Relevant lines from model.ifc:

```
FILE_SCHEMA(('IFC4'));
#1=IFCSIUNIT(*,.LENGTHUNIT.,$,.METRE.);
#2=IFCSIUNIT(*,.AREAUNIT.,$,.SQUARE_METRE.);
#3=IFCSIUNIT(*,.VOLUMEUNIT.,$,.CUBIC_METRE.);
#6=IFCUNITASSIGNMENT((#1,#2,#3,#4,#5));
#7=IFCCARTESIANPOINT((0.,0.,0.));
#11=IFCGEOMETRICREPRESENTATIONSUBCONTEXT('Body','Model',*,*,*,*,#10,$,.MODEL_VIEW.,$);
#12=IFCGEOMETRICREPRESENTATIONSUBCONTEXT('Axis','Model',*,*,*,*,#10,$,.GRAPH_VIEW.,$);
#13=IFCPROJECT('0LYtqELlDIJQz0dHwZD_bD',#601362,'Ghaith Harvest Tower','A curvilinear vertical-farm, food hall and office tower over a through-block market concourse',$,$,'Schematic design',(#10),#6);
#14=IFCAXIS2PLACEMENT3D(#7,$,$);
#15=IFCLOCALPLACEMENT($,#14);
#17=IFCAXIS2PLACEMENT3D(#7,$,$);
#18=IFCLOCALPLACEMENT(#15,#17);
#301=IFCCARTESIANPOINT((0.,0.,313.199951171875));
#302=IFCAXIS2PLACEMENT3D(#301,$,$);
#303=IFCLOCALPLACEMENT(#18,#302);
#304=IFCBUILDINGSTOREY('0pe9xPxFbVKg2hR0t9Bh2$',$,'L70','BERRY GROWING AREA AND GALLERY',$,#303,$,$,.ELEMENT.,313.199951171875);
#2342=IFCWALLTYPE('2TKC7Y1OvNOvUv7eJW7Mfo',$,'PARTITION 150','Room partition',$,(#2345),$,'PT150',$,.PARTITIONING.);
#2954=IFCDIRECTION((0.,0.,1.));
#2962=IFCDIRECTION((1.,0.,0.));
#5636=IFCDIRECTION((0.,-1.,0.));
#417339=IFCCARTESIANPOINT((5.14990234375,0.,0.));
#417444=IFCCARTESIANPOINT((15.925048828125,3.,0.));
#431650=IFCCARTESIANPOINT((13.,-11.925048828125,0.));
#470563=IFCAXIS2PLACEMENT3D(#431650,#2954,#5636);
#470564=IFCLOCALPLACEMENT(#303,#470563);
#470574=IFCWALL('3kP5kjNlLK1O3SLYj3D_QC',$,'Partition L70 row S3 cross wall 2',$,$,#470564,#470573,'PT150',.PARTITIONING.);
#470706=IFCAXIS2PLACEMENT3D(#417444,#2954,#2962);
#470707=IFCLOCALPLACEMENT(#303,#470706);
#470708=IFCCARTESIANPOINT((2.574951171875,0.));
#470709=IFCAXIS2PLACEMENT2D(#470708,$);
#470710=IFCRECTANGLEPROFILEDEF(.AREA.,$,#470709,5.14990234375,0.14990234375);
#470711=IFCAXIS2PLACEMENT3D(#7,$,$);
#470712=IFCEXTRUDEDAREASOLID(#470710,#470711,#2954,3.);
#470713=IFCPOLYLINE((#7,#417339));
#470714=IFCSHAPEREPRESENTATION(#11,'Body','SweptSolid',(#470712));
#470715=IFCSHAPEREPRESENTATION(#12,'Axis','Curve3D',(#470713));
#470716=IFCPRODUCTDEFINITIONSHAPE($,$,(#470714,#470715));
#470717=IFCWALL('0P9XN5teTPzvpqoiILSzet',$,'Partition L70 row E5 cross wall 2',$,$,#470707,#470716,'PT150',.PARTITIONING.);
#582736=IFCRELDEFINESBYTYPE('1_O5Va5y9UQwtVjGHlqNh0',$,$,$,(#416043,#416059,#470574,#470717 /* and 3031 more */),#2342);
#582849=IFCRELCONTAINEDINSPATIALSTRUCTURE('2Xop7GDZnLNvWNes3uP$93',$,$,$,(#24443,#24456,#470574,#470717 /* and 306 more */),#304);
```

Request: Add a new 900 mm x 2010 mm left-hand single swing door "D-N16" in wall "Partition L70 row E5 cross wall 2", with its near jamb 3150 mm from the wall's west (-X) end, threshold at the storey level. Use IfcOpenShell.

```python
import numpy as np
import ifcopenshell
import ifcopenshell.api.feature
import ifcopenshell.api.geometry
import ifcopenshell.api.root
import ifcopenshell.api.spatial
import ifcopenshell.geom
import ifcopenshell.util.element
import ifcopenshell.util.placement
import ifcopenshell.util.representation
import ifcopenshell.util.shape
import ifcopenshell.util.unit

model = ifcopenshell.open("model.ifc")
unit_scale = ifcopenshell.util.unit.calculate_unit_scale(model)
settings = ifcopenshell.geom.settings()


def volume(element):
    """Net volume in cubic metres, openings subtracted."""
    shape = ifcopenshell.geom.create_shape(settings, element)
    return ifcopenshell.util.shape.get_volume(shape.geometry)


wall = model.by_id(470717)
storey = ifcopenshell.util.element.get_container(wall, ifc_class="IfcBuildingStorey")
context = ifcopenshell.util.representation.get_context(model, "Model", "Body", "MODEL_VIEW")
before = volume(wall)

width, height, from_end, sill = 0.9, 2.01, 3.15, 0.0  # metres

# The wall runs along its own X axis, and the end named is its -X end.
wall_shape = ifcopenshell.geom.create_shape(settings, wall)
x, y, z = ifcopenshell.util.shape.get_vertices(wall_shape.geometry).T
start = x.min() + from_end
face, thickness = float(y.min()), float(y.max() - y.min())
wall_matrix = ifcopenshell.util.placement.get_local_placement(wall.ObjectPlacement)
level = ifcopenshell.util.placement.get_local_placement(storey.ObjectPlacement)[2, 3]


def in_wall(x, y):
    """Placement at x, y metres in the wall's axes, at sill height."""
    matrix = wall_matrix.copy()
    matrix[:, 3] = wall_matrix @ np.array([x / unit_scale, y / unit_scale, 0.0, 1.0])
    matrix[2, 3] = level + sill / unit_scale
    return matrix


# Opening: a box that overshoots both wall faces by 50 mm.
opening = ifcopenshell.api.root.create_entity(model, ifc_class="IfcOpeningElement", predefined_type="OPENING")
box = ifcopenshell.api.geometry.add_wall_representation(
    model, context=context, length=width, height=height, thickness=thickness + 0.1
)
ifcopenshell.api.geometry.assign_representation(model, product=opening, representation=box)
ifcopenshell.api.geometry.edit_object_placement(model, product=opening, matrix=in_wall(start, face - 0.05), is_si=False)
ifcopenshell.api.feature.add_feature(model, feature=opening, element=wall)

door = ifcopenshell.api.root.create_entity(model, ifc_class="IfcDoor", name="D-N16", predefined_type="DOOR")
door.OverallWidth, door.OverallHeight = width / unit_scale, height / unit_scale
door.OperationType = "SINGLE_SWING_LEFT"
body = ifcopenshell.api.geometry.add_door_representation(
    model,
    context=context,
    overall_width=door.OverallWidth,
    overall_height=door.OverallHeight,
    operation_type="SINGLE_SWING_LEFT",
    lining_properties={"LiningDepth": thickness / unit_scale, "ThresholdDepth": thickness / unit_scale},
)
ifcopenshell.api.geometry.assign_representation(model, product=door, representation=body)
ifcopenshell.api.spatial.assign_container(model, products=[door], relating_structure=storey)
ifcopenshell.api.feature.add_filling(model, opening=opening, element=door)

# The lining spans the wall, so the door starts at the wall face.
ifcopenshell.api.geometry.edit_object_placement(model, product=door, matrix=in_wall(start, face), is_si=False)

after = volume(wall)

print(f"wall volume {before:.3f} -> {after:.3f} m3")

model.write("model_edited.ifc")
```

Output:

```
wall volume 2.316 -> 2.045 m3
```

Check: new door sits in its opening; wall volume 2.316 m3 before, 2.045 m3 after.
